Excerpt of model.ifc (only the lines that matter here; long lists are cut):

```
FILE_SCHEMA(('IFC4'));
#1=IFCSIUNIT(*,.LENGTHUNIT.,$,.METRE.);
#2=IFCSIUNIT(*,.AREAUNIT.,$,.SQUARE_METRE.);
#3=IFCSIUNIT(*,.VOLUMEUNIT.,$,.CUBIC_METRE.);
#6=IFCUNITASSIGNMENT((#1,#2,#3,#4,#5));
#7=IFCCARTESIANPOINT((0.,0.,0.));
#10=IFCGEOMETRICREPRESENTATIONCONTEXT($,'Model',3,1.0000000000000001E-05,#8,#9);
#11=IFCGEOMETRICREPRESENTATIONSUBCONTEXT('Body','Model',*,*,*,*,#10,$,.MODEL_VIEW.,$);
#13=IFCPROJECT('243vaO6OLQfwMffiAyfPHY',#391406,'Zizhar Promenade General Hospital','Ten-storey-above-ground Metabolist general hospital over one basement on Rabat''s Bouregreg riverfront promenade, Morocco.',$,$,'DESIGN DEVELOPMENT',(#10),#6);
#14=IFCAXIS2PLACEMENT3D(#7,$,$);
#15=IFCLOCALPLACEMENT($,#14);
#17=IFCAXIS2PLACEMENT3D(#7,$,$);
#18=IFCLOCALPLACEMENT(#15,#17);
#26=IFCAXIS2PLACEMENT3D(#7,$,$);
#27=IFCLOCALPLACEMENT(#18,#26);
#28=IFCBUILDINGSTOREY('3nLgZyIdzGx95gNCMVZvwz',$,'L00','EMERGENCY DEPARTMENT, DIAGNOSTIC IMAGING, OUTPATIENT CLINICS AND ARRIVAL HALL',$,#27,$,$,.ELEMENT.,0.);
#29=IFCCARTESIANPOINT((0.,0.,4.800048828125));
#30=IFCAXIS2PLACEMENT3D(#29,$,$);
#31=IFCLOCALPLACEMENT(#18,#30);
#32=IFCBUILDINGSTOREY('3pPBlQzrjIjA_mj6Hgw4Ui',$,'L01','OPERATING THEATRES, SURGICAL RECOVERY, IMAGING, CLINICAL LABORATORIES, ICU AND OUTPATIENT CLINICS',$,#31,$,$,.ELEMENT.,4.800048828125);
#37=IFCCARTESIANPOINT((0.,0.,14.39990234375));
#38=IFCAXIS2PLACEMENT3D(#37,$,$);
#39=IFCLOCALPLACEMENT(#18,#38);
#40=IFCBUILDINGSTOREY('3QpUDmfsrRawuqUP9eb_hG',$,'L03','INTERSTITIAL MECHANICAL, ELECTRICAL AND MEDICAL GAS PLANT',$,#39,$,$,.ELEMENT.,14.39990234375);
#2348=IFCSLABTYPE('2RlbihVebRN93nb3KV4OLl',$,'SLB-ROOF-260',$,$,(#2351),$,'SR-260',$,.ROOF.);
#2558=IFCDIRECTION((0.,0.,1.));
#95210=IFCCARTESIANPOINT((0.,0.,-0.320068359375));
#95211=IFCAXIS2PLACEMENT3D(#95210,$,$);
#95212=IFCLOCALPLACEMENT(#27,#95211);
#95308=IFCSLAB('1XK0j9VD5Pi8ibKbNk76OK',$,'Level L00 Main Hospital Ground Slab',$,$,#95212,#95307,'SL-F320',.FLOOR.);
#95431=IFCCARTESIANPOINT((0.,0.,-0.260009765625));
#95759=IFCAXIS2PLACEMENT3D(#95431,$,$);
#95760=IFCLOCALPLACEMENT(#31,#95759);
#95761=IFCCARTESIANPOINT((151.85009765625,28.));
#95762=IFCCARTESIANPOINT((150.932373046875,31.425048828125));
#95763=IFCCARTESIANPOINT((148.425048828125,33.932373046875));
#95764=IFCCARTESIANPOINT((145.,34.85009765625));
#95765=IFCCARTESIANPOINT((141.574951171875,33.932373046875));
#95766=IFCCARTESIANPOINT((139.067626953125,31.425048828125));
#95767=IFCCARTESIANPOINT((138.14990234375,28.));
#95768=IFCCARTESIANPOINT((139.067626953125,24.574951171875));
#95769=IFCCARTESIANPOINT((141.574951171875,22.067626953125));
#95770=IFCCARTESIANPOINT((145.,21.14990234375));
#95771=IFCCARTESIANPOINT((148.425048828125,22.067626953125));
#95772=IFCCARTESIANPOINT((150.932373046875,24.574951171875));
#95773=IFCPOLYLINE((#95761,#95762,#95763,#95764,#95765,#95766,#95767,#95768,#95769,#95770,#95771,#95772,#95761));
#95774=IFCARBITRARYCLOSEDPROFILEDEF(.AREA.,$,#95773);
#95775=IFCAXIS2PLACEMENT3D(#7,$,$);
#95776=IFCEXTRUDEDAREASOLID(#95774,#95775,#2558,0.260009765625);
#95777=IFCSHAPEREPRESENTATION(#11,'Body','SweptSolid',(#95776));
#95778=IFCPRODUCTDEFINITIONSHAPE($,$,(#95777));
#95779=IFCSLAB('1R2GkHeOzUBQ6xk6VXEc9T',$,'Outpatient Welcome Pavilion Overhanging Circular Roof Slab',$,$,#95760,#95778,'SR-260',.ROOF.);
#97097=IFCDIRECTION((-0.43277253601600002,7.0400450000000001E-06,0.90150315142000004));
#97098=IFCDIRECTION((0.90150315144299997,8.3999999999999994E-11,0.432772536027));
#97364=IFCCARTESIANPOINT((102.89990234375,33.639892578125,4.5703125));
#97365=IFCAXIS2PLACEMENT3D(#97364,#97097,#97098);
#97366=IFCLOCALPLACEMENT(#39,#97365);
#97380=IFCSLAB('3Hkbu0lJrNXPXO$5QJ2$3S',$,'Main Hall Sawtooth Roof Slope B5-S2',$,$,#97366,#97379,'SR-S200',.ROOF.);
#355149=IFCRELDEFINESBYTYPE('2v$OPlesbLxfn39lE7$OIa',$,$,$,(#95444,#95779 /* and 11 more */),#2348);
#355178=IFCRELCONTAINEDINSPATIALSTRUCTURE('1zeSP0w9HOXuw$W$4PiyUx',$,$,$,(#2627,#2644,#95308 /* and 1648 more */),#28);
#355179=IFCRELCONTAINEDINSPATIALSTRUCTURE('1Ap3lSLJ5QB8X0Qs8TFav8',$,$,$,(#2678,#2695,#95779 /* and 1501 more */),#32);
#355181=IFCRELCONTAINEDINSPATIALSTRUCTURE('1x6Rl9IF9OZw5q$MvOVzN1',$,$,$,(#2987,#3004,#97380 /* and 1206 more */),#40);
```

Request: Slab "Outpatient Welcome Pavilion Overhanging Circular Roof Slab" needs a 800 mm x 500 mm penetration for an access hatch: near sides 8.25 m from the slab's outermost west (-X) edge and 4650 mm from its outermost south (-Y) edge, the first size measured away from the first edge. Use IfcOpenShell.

```python
import numpy as np
import ifcopenshell
import ifcopenshell.api.feature
import ifcopenshell.api.geometry
import ifcopenshell.api.root
import ifcopenshell.geom
import ifcopenshell.util.placement
import ifcopenshell.util.representation
import ifcopenshell.util.shape
import ifcopenshell.util.unit

model = ifcopenshell.open("model.ifc")
unit_scale = ifcopenshell.util.unit.calculate_unit_scale(model)
settings = ifcopenshell.geom.settings()


def volume(element):
    """Net volume in cubic metres, openings subtracted."""
    shape = ifcopenshell.geom.create_shape(settings, element)
    return ifcopenshell.util.shape.get_volume(shape.geometry)


slab = model.by_guid("1R2GkHeOzUBQ6xk6VXEc9T")
before = volume(slab)

# Extent in the slab's own axes, in metres. The edges named are its -X and -Y sides.
slab_shape = ifcopenshell.geom.create_shape(settings, slab)
vertices = ifcopenshell.util.shape.get_vertices(slab_shape.geometry)
x_min, y_min, bottom = vertices.min(axis=0)
top = vertices[:, 2].max()

opening = ifcopenshell.api.root.create_entity(model, ifc_class="IfcOpeningElement", name="Access hatch opening", predefined_type="OPENING")
context = ifcopenshell.util.representation.get_context(model, "Model", "Body", "MODEL_VIEW")
width, depth = 0.8, 0.5
outline = [(0.0, 0.0), (width, 0.0), (width, depth), (0.0, depth), (0.0, 0.0)]
# Overshoot both faces by 50 mm so the cut is clean.
shape = ifcopenshell.api.geometry.add_slab_representation(
    model, context=context, depth=top - bottom + 0.1, polyline=outline
)
ifcopenshell.api.geometry.assign_representation(model, product=opening, representation=shape)

matrix = ifcopenshell.util.placement.get_local_placement(slab.ObjectPlacement)
matrix[:, 3] = matrix @ np.append(np.array([x_min + 8.25, y_min + 4.65, bottom - 0.05]) / unit_scale, 1.0)
ifcopenshell.api.geometry.edit_object_placement(model, product=opening, matrix=matrix, is_si=False)
ifcopenshell.api.feature.add_feature(model, feature=opening, element=slab)

after = volume(slab)

print(f"slab volume {before:.3f} -> {after:.3f} m3")

model.write("model_v2.ifc")
```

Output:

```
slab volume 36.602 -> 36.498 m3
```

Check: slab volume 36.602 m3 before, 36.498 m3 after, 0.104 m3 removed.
